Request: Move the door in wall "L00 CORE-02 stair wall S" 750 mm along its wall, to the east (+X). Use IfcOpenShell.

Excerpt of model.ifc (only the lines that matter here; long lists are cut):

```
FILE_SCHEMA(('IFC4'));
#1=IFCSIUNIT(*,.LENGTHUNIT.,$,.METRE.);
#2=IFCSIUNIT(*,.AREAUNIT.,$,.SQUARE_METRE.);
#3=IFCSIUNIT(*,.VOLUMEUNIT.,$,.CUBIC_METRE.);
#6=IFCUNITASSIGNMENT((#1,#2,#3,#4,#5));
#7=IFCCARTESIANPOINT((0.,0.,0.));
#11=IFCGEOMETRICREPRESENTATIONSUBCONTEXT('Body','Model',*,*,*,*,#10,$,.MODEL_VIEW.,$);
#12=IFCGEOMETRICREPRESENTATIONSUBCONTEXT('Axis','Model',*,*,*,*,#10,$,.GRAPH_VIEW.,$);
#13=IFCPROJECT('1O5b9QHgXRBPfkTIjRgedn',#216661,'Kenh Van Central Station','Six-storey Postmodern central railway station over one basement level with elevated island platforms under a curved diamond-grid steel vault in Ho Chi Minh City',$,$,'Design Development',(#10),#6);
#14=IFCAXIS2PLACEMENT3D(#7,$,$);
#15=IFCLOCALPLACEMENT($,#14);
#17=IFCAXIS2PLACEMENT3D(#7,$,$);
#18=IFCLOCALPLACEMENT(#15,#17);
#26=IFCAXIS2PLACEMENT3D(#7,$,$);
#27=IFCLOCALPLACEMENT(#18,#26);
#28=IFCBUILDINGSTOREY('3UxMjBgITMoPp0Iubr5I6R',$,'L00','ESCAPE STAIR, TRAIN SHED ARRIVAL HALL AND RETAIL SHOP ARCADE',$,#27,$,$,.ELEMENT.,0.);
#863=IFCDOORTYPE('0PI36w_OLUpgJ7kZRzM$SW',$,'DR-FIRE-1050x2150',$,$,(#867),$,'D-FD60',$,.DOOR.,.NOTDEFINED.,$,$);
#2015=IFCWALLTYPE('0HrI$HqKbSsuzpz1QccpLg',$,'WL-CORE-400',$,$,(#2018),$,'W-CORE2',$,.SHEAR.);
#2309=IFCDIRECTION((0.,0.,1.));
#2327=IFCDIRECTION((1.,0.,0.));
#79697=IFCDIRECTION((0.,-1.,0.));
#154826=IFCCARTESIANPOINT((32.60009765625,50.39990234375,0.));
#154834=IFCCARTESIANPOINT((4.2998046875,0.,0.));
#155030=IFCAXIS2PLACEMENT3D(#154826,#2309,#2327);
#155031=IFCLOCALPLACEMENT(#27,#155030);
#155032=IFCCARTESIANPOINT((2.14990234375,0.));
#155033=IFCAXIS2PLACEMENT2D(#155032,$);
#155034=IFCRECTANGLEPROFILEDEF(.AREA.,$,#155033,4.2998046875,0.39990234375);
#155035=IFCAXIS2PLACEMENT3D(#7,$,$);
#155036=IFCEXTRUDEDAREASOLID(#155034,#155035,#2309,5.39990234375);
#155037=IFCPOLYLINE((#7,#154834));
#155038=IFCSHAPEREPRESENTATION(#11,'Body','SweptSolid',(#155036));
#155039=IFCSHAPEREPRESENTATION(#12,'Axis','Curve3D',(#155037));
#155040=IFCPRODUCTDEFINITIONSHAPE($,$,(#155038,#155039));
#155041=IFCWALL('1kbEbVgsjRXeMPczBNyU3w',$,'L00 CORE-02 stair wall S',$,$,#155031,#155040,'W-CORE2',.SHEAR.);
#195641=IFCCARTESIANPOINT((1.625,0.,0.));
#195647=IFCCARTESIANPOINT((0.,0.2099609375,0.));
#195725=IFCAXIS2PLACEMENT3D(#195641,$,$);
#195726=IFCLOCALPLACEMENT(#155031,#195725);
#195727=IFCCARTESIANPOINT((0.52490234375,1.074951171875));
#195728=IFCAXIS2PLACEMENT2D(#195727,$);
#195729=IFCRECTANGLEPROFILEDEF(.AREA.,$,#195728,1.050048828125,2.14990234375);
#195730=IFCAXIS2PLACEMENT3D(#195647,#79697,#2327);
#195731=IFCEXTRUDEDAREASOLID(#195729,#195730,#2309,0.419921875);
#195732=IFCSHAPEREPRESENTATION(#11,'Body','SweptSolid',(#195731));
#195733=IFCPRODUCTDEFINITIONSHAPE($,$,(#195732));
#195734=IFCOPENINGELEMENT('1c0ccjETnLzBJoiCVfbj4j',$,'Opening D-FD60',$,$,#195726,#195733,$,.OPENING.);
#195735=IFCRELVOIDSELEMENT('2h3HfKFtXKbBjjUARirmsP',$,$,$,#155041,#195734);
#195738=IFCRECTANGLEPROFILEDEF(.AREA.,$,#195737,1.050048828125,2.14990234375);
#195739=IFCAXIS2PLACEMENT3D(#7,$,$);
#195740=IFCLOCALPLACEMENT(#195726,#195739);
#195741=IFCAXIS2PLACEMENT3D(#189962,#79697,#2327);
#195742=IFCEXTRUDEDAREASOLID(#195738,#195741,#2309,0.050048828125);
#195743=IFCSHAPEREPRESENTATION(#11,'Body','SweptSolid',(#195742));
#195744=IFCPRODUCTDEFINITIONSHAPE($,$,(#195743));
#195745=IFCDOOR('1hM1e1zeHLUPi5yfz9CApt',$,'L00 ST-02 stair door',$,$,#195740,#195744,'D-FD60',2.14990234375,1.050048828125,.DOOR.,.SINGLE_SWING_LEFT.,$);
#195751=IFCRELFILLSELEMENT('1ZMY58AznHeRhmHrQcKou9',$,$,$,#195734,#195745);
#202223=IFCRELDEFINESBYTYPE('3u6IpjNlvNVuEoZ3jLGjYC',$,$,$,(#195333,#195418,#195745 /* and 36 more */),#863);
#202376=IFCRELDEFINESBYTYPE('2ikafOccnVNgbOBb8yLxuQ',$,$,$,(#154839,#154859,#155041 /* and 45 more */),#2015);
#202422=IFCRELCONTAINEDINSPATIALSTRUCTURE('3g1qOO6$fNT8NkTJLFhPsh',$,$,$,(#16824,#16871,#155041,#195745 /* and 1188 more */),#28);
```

```python
import ifcopenshell
import ifcopenshell.api.geometry
import ifcopenshell.util.placement
import ifcopenshell.util.unit

model = ifcopenshell.open("model.ifc")
unit_scale = ifcopenshell.util.unit.calculate_unit_scale(model)

door = model.by_guid("1hM1e1zeHLUPi5yfz9CApt")
opening = door.FillsVoids[0].RelatingOpeningElement
wall = opening.VoidsElements[0].RelatingBuildingElement

wall_matrix = ifcopenshell.util.placement.get_local_placement(wall.ObjectPlacement)
shift = wall_matrix[:3, 0] * 0.75 / unit_scale
before = ifcopenshell.util.placement.get_local_placement(door.ObjectPlacement)[:3, 3].copy()

# The door is placed relative to its opening, so it follows when the opening moves.
matrix = ifcopenshell.util.placement.get_local_placement(opening.ObjectPlacement)
matrix[:3, 3] += shift
ifcopenshell.api.geometry.edit_object_placement(
    model, product=opening, matrix=matrix, is_si=False, should_transform_children=True
)

after = ifcopenshell.util.placement.get_local_placement(door.ObjectPlacement)[:3, 3]
print("door moved by", (after - before).round(3) + 0.0)

model.write("model_updated.ifc")
```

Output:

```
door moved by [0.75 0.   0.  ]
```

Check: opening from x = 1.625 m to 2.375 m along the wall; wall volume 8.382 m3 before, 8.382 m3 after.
